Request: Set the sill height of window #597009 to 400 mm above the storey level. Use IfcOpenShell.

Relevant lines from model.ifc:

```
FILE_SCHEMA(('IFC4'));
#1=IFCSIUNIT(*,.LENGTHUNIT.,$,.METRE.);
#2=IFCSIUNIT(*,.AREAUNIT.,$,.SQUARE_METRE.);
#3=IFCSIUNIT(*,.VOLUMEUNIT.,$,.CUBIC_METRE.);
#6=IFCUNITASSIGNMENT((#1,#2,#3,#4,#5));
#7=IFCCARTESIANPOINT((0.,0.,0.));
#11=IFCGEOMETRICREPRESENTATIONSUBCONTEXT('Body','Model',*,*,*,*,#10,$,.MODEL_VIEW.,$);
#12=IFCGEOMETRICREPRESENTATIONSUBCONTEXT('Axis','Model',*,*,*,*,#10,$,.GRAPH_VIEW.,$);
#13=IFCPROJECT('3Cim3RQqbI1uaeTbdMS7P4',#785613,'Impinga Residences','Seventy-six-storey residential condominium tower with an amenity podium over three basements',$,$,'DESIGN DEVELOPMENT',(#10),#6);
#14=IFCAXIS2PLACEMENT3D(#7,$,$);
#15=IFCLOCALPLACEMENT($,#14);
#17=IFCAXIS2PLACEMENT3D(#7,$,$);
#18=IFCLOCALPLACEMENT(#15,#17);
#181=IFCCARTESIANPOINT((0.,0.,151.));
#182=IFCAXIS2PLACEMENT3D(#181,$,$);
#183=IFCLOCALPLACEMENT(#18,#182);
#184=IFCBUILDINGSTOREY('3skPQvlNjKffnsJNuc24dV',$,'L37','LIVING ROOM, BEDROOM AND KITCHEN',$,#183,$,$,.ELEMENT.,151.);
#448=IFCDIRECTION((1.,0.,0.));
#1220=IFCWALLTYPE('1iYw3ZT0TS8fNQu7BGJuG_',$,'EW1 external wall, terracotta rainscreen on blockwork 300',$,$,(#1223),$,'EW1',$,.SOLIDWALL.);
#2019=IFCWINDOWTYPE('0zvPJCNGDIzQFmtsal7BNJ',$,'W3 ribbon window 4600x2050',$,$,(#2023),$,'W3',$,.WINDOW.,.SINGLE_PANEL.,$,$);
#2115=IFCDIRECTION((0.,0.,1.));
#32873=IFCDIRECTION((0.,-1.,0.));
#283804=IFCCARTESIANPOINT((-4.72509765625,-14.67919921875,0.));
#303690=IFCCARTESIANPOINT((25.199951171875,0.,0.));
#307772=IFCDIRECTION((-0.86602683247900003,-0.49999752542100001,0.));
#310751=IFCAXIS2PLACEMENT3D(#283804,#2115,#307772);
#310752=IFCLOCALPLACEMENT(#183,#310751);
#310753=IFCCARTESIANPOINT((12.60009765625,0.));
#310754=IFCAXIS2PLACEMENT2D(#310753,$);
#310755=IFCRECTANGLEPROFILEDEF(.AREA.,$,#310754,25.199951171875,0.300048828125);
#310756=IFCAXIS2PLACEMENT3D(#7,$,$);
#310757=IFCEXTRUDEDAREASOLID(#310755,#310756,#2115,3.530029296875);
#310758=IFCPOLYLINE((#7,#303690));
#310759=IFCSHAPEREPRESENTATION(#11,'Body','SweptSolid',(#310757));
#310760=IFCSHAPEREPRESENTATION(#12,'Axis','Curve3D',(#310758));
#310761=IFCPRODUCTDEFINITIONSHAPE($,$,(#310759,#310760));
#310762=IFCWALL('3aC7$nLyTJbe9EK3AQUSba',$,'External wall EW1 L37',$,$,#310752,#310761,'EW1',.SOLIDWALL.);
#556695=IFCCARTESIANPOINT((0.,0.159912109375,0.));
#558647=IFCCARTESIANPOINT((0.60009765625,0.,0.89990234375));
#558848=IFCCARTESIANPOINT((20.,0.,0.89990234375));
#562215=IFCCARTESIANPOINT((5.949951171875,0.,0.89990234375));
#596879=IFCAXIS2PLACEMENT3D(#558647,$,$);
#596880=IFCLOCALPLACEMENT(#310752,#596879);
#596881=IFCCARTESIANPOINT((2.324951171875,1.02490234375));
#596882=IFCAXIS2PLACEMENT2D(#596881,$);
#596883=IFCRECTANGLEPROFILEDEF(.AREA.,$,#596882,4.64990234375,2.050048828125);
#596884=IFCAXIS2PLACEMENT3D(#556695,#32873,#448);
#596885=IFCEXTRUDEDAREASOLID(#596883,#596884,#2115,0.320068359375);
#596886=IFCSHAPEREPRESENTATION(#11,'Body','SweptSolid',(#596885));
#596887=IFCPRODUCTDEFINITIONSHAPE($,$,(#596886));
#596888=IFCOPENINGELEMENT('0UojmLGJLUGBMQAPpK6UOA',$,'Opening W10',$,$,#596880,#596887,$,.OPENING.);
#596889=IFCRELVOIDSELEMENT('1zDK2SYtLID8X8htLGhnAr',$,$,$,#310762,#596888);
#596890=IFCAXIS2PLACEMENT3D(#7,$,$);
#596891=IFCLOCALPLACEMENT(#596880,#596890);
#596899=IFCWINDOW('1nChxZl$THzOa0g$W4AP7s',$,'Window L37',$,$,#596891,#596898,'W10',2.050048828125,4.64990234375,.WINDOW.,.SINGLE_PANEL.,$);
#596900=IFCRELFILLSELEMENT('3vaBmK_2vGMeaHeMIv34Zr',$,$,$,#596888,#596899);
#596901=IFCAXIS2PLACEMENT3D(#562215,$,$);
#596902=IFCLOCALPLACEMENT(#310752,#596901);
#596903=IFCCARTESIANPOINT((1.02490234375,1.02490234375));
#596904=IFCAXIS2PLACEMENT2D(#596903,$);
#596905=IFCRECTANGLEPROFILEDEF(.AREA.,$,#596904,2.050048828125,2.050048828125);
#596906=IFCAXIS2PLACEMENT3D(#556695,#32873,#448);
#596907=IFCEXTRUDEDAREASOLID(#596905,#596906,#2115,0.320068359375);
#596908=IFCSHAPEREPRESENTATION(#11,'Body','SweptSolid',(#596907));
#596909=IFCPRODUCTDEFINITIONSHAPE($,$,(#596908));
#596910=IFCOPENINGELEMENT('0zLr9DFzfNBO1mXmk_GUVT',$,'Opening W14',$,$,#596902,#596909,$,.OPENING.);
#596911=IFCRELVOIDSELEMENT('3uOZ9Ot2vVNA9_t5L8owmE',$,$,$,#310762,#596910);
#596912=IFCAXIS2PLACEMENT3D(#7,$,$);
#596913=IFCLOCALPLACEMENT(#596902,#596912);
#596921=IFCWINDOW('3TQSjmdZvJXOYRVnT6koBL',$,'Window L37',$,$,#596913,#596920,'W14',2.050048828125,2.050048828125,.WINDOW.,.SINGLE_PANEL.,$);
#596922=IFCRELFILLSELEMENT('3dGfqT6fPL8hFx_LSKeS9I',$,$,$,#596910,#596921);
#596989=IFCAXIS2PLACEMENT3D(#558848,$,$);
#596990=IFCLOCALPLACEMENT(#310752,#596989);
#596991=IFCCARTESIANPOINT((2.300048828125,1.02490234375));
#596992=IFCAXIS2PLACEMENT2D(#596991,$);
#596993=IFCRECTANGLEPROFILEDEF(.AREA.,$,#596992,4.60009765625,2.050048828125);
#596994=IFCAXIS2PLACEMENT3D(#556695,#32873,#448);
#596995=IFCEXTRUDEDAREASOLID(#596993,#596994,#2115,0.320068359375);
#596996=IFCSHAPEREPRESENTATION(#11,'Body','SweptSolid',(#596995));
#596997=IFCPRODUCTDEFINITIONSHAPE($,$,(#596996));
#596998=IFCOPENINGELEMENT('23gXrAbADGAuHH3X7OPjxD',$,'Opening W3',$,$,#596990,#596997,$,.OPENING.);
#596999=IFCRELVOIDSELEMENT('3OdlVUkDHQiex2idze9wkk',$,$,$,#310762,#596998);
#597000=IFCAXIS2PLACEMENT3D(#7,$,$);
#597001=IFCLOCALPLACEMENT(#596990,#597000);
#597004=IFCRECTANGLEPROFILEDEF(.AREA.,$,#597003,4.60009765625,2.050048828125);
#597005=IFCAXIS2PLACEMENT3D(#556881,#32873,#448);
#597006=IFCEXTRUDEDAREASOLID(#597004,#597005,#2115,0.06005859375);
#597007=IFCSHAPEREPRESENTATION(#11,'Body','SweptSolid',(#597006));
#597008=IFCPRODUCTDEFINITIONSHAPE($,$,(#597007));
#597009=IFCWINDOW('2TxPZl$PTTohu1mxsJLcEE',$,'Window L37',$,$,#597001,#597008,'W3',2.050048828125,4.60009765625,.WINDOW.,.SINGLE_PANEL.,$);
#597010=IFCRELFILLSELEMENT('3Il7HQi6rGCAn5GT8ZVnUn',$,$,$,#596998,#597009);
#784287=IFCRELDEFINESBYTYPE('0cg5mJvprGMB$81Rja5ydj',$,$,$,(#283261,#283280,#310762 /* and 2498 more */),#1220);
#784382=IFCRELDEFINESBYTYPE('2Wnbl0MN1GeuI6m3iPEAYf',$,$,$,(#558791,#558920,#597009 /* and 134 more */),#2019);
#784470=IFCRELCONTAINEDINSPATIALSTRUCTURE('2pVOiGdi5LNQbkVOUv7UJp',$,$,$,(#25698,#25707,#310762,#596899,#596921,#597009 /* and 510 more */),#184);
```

```python
import numpy as np
import ifcopenshell
import ifcopenshell.api.geometry
import ifcopenshell.geom
import ifcopenshell.util.element
import ifcopenshell.util.placement
import ifcopenshell.util.shape
import ifcopenshell.util.unit

model = ifcopenshell.open("model.ifc")
unit_scale = ifcopenshell.util.unit.calculate_unit_scale(model)

window = model.by_guid("2TxPZl$PTTohu1mxsJLcEE")
opening = window.FillsVoids[0].RelatingOpeningElement
storey = ifcopenshell.util.element.get_container(window, ifc_class="IfcBuildingStorey")
level = ifcopenshell.util.placement.get_local_placement(storey.ObjectPlacement)[2, 3]

# The opening's origin need not be at the sill, so measure its lowest point.
shape = ifcopenshell.geom.create_shape(ifcopenshell.geom.settings(), opening)
bottom = ifcopenshell.util.shape.get_shape_bottom_elevation(shape, shape.geometry) / unit_scale
dz = level + 0.4 - bottom

shift = np.array([0.0, 0.0, dz])
# The window is placed relative to its opening, so it follows when the opening moves.
matrix = ifcopenshell.util.placement.get_local_placement(opening.ObjectPlacement)
matrix[:3, 3] += shift
ifcopenshell.api.geometry.edit_object_placement(
    model, product=opening, matrix=matrix, is_si=False, should_transform_children=True
)

print(f"moved by {dz * unit_scale:+.3f} m")

model.write("model_updated.ifc")
```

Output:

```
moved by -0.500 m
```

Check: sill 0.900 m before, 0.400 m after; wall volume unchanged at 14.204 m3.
